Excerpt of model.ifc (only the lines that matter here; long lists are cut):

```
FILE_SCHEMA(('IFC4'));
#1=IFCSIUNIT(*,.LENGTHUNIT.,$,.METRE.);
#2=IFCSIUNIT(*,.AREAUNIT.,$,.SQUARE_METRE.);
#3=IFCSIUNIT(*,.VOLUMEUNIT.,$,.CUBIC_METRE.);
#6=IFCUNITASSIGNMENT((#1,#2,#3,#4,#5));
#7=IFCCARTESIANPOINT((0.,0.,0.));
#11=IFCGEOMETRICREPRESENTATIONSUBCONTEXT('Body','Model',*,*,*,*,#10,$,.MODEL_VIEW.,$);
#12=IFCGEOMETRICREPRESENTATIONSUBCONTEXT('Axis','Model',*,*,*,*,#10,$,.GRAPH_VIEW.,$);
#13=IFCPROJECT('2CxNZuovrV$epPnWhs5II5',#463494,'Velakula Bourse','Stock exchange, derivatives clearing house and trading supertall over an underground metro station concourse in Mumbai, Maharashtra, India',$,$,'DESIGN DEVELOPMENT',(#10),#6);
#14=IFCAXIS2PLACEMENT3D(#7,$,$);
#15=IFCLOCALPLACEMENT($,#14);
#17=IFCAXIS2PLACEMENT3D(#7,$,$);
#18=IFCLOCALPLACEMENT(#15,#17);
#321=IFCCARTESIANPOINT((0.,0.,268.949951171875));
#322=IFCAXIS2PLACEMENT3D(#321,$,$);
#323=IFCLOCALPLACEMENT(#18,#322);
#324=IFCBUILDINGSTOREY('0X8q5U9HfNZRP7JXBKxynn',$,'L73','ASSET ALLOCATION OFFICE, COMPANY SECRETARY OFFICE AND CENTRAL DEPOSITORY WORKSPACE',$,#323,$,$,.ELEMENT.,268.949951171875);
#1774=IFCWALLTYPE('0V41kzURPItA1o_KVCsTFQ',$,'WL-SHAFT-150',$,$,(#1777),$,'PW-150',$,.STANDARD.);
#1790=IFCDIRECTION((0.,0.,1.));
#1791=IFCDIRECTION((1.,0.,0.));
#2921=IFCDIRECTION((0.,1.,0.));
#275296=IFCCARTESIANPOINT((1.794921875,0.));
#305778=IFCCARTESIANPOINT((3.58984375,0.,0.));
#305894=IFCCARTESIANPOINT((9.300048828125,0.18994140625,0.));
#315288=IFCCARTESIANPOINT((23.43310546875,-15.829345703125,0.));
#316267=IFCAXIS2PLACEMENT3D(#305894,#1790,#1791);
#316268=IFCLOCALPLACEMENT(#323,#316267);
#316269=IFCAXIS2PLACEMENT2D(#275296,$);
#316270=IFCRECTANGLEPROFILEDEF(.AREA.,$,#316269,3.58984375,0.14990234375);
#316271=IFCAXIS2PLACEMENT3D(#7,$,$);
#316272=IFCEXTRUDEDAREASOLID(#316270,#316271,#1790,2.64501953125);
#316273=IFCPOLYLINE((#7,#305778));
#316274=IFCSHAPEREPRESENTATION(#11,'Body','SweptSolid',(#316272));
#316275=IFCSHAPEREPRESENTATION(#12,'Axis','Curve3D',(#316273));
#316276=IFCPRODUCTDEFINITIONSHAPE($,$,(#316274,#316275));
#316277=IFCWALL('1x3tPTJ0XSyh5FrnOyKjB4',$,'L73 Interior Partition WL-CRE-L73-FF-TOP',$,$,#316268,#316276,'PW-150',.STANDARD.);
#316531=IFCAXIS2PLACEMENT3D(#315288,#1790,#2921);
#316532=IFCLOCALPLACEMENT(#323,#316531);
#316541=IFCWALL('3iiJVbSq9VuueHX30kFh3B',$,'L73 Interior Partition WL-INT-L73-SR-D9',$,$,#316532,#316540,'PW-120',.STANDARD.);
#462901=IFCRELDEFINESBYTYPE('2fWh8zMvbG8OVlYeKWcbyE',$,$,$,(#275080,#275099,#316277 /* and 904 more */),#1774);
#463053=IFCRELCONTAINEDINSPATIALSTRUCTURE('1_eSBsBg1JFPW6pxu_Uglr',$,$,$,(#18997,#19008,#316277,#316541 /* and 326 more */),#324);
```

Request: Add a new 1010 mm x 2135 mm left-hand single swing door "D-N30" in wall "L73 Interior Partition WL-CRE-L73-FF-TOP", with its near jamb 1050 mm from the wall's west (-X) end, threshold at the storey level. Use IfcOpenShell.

```python
import numpy as np
import ifcopenshell
import ifcopenshell.api.feature
import ifcopenshell.api.geometry
import ifcopenshell.api.root
import ifcopenshell.api.spatial
import ifcopenshell.geom
import ifcopenshell.util.element
import ifcopenshell.util.placement
import ifcopenshell.util.representation
import ifcopenshell.util.shape
import ifcopenshell.util.unit

model = ifcopenshell.open("model.ifc")
unit_scale = ifcopenshell.util.unit.calculate_unit_scale(model)
settings = ifcopenshell.geom.settings()


def volume(element):
    """Net volume in cubic metres, openings subtracted."""
    shape = ifcopenshell.geom.create_shape(settings, element)
    return ifcopenshell.util.shape.get_volume(shape.geometry)


wall = model.by_guid("1x3tPTJ0XSyh5FrnOyKjB4")
storey = ifcopenshell.util.element.get_container(wall, ifc_class="IfcBuildingStorey")
context = ifcopenshell.util.representation.get_context(model, "Model", "Body", "MODEL_VIEW")
before = volume(wall)

width, height, from_end, sill = 1.01, 2.135, 1.05, 0.0  # metres

# The wall runs along its own X axis, and the end named is its -X end.
wall_shape = ifcopenshell.geom.create_shape(settings, wall)
x, y, z = ifcopenshell.util.shape.get_vertices(wall_shape.geometry).T
start = x.min() + from_end
face, thickness = float(y.min()), float(y.max() - y.min())
wall_matrix = ifcopenshell.util.placement.get_local_placement(wall.ObjectPlacement)
level = ifcopenshell.util.placement.get_local_placement(storey.ObjectPlacement)[2, 3]


def in_wall(x, y):
    """Placement at x, y metres in the wall's axes, at sill height."""
    matrix = wall_matrix.copy()
    matrix[:, 3] = wall_matrix @ np.array([x / unit_scale, y / unit_scale, 0.0, 1.0])
    matrix[2, 3] = level + sill / unit_scale
    return matrix


# Opening: a box that overshoots both wall faces by 50 mm.
opening = ifcopenshell.api.root.create_entity(model, ifc_class="IfcOpeningElement", predefined_type="OPENING")
box = ifcopenshell.api.geometry.add_wall_representation(
    model, context=context, length=width, height=height, thickness=thickness + 0.1
)
ifcopenshell.api.geometry.assign_representation(model, product=opening, representation=box)
ifcopenshell.api.geometry.edit_object_placement(model, product=opening, matrix=in_wall(start, face - 0.05), is_si=False)
ifcopenshell.api.feature.add_feature(model, feature=opening, element=wall)

door = ifcopenshell.api.root.create_entity(model, ifc_class="IfcDoor", name="D-N30", predefined_type="DOOR")
door.OverallWidth, door.OverallHeight = width / unit_scale, height / unit_scale
door.OperationType = "SINGLE_SWING_LEFT"
body = ifcopenshell.api.geometry.add_door_representation(
    model,
    context=context,
    overall_width=door.OverallWidth,
    overall_height=door.OverallHeight,
    operation_type="SINGLE_SWING_LEFT",
    lining_properties={"LiningDepth": thickness / unit_scale, "ThresholdDepth": thickness / unit_scale},
)
ifcopenshell.api.geometry.assign_representation(model, product=door, representation=body)
ifcopenshell.api.spatial.assign_container(model, products=[door], relating_structure=storey)
ifcopenshell.api.feature.add_filling(model, opening=opening, element=door)

# The lining spans the wall, so the door starts at the wall face.
ifcopenshell.api.geometry.edit_object_placement(model, product=door, matrix=in_wall(start, face), is_si=False)

after = volume(wall)

print(f"wall volume {before:.3f} -> {after:.3f} m3")

model.write("model_rev.ifc")
```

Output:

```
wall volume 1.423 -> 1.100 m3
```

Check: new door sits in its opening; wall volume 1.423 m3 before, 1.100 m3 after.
